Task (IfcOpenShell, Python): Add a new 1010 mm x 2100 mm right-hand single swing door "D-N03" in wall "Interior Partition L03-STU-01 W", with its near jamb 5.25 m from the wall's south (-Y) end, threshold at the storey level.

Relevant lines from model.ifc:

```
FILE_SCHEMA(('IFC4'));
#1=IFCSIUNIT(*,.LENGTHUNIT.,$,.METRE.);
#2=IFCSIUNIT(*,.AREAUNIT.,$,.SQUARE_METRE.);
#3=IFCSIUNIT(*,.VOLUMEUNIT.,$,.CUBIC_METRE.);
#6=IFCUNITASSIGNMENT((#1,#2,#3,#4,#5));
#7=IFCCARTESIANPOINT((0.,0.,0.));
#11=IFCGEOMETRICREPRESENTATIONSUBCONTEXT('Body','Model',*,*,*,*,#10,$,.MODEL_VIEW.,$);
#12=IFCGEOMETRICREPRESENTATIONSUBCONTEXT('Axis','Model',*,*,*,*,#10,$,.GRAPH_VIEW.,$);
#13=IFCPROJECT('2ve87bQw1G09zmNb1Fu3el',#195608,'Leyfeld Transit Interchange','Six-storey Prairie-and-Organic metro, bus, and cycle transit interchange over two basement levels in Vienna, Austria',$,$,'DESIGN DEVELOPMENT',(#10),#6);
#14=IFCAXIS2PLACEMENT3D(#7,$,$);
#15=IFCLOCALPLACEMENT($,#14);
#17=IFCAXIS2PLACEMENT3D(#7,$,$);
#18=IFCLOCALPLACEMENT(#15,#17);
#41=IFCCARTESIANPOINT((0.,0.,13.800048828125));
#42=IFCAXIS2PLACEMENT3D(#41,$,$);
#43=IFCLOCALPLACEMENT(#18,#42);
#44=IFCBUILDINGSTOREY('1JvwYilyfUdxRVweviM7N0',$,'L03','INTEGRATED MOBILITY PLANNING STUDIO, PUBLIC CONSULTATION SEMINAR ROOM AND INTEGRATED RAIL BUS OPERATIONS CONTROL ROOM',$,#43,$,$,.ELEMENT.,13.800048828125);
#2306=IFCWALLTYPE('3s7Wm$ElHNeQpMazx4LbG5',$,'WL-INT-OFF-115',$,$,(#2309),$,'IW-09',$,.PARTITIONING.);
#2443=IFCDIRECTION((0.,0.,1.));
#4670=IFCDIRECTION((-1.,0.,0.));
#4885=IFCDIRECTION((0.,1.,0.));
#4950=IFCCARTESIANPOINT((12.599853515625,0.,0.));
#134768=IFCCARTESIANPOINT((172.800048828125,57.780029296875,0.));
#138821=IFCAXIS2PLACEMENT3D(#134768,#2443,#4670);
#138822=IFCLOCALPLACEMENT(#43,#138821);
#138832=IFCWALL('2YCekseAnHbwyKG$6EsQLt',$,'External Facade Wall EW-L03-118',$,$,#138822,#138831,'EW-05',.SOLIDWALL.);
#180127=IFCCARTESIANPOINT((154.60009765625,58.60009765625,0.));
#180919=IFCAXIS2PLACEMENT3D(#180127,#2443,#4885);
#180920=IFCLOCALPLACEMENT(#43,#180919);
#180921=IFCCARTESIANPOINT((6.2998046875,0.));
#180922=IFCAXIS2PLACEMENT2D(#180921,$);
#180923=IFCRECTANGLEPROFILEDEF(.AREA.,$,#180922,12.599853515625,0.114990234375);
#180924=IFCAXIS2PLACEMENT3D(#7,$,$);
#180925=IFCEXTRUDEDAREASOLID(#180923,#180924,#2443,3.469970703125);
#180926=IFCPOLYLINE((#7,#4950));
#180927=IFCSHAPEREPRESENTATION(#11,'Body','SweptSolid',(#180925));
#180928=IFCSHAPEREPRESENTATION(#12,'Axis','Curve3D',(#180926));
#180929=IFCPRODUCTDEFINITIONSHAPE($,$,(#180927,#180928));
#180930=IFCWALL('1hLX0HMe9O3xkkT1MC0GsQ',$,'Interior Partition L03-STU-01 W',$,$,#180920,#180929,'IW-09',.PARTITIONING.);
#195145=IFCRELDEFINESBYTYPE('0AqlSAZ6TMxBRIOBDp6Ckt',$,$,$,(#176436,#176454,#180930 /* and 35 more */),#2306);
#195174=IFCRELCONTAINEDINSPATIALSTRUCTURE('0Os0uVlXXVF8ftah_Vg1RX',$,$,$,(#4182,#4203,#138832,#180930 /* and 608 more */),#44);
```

```python
import numpy as np
import ifcopenshell
import ifcopenshell.api.feature
import ifcopenshell.api.geometry
import ifcopenshell.api.root
import ifcopenshell.api.spatial
import ifcopenshell.geom
import ifcopenshell.util.element
import ifcopenshell.util.placement
import ifcopenshell.util.representation
import ifcopenshell.util.shape
import ifcopenshell.util.unit

model = ifcopenshell.open("model.ifc")
unit_scale = ifcopenshell.util.unit.calculate_unit_scale(model)
settings = ifcopenshell.geom.settings()


def volume(element):
    """Net volume in cubic metres, openings subtracted."""
    shape = ifcopenshell.geom.create_shape(settings, element)
    return ifcopenshell.util.shape.get_volume(shape.geometry)


wall = model.by_guid("1hLX0HMe9O3xkkT1MC0GsQ")
storey = ifcopenshell.util.element.get_container(wall, ifc_class="IfcBuildingStorey")
context = ifcopenshell.util.representation.get_context(model, "Model", "Body", "MODEL_VIEW")
before = volume(wall)

width, height, from_end, sill = 1.01, 2.1, 5.25, 0.0  # metres

# The wall runs along its own X axis, and the end named is its -X end.
wall_shape = ifcopenshell.geom.create_shape(settings, wall)
x, y, z = ifcopenshell.util.shape.get_vertices(wall_shape.geometry).T
start = x.min() + from_end
face, thickness = float(y.min()), float(y.max() - y.min())
wall_matrix = ifcopenshell.util.placement.get_local_placement(wall.ObjectPlacement)
level = ifcopenshell.util.placement.get_local_placement(storey.ObjectPlacement)[2, 3]


def in_wall(x, y):
    """Placement at x, y metres in the wall's axes, at sill height."""
    matrix = wall_matrix.copy()
    matrix[:, 3] = wall_matrix @ np.array([x / unit_scale, y / unit_scale, 0.0, 1.0])
    matrix[2, 3] = level + sill / unit_scale
    return matrix


# Opening: a box that overshoots both wall faces by 50 mm.
opening = ifcopenshell.api.root.create_entity(model, ifc_class="IfcOpeningElement", predefined_type="OPENING")
box = ifcopenshell.api.geometry.add_wall_representation(
    model, context=context, length=width, height=height, thickness=thickness + 0.1
)
ifcopenshell.api.geometry.assign_representation(model, product=opening, representation=box)
ifcopenshell.api.geometry.edit_object_placement(model, product=opening, matrix=in_wall(start, face - 0.05), is_si=False)
ifcopenshell.api.feature.add_feature(model, feature=opening, element=wall)

door = ifcopenshell.api.root.create_entity(model, ifc_class="IfcDoor", name="D-N03", predefined_type="DOOR")
door.OverallWidth, door.OverallHeight = width / unit_scale, height / unit_scale
door.OperationType = "SINGLE_SWING_RIGHT"
body = ifcopenshell.api.geometry.add_door_representation(
    model,
    context=context,
    overall_width=door.OverallWidth,
    overall_height=door.OverallHeight,
    operation_type="SINGLE_SWING_RIGHT",
    lining_properties={"LiningDepth": thickness / unit_scale, "ThresholdDepth": thickness / unit_scale},
)
ifcopenshell.api.geometry.assign_representation(model, product=door, representation=body)
ifcopenshell.api.spatial.assign_container(model, products=[door], relating_structure=storey)
ifcopenshell.api.feature.add_filling(model, opening=opening, element=door)

# The lining spans the wall, so the door starts at the wall face.
ifcopenshell.api.geometry.edit_object_placement(model, product=door, matrix=in_wall(start, face), is_si=False)

after = volume(wall)

print(f"wall volume {before:.3f} -> {after:.3f} m3")

model.write("model_updated.ifc")
```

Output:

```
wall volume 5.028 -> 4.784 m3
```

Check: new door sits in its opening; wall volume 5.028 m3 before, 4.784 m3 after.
